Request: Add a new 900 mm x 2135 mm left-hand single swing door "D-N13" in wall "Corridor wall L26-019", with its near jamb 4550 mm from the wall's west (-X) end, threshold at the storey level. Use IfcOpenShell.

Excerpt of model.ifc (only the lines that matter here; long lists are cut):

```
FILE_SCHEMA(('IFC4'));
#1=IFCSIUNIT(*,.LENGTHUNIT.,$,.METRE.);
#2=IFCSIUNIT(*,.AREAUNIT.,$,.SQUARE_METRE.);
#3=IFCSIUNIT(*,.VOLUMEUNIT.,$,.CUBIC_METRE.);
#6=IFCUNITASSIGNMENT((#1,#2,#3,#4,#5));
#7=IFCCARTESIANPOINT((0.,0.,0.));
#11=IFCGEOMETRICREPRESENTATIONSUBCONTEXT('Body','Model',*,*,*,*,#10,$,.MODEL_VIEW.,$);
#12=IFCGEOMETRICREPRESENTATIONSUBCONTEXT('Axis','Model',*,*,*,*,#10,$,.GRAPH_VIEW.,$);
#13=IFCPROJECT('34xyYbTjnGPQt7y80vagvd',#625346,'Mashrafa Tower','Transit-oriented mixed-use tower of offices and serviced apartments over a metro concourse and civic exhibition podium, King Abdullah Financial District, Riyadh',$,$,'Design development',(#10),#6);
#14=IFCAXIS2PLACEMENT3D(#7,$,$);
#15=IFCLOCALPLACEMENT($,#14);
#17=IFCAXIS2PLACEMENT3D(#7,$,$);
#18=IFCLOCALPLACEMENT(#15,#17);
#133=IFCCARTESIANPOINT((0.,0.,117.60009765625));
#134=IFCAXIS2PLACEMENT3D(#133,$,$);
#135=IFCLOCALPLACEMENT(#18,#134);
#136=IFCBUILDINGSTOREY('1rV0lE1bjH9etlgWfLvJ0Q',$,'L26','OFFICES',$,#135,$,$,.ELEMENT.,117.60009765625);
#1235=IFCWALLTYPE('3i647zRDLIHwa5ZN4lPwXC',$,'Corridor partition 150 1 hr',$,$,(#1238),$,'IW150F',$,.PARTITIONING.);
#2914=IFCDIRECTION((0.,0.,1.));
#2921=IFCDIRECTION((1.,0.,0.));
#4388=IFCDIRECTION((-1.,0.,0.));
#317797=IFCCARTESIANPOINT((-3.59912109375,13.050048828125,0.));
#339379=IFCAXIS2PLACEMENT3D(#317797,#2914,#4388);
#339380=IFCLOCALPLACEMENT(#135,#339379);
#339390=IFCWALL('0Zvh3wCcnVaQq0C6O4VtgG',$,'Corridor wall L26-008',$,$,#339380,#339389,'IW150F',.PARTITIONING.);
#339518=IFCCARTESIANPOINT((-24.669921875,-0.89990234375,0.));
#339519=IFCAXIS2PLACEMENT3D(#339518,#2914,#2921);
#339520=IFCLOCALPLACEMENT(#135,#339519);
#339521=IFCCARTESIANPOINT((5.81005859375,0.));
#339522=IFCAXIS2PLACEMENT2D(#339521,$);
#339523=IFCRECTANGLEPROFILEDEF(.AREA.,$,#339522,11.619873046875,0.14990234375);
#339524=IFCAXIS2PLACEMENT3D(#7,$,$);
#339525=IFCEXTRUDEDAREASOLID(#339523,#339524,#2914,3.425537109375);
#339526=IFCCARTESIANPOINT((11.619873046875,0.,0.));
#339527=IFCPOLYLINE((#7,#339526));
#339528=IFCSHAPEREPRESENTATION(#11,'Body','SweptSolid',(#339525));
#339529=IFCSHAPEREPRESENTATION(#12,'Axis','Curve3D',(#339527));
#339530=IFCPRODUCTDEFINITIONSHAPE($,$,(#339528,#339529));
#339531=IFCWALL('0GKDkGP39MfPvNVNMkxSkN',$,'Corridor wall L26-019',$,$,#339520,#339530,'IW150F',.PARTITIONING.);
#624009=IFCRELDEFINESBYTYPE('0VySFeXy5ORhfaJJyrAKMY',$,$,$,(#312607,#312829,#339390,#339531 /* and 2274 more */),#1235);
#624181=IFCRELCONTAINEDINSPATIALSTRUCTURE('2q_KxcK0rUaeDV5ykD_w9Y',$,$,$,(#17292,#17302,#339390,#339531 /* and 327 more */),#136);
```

```python
import numpy as np
import ifcopenshell
import ifcopenshell.api.feature
import ifcopenshell.api.geometry
import ifcopenshell.api.root
import ifcopenshell.api.spatial
import ifcopenshell.geom
import ifcopenshell.util.element
import ifcopenshell.util.placement
import ifcopenshell.util.representation
import ifcopenshell.util.shape
import ifcopenshell.util.unit

model = ifcopenshell.open("model.ifc")
unit_scale = ifcopenshell.util.unit.calculate_unit_scale(model)
settings = ifcopenshell.geom.settings()


def volume(element):
    """Net volume in cubic metres, openings subtracted."""
    shape = ifcopenshell.geom.create_shape(settings, element)
    return ifcopenshell.util.shape.get_volume(shape.geometry)


wall = model.by_guid("0GKDkGP39MfPvNVNMkxSkN")
storey = ifcopenshell.util.element.get_container(wall, ifc_class="IfcBuildingStorey")
context = ifcopenshell.util.representation.get_context(model, "Model", "Body", "MODEL_VIEW")
before = volume(wall)

width, height, from_end, sill = 0.9, 2.135, 4.55, 0.0  # metres

# The wall runs along its own X axis, and the end named is its -X end.
wall_shape = ifcopenshell.geom.create_shape(settings, wall)
x, y, z = ifcopenshell.util.shape.get_vertices(wall_shape.geometry).T
start = x.min() + from_end
face, thickness = float(y.min()), float(y.max() - y.min())
wall_matrix = ifcopenshell.util.placement.get_local_placement(wall.ObjectPlacement)
level = ifcopenshell.util.placement.get_local_placement(storey.ObjectPlacement)[2, 3]


def in_wall(x, y):
    """Placement at x, y metres in the wall's axes, at sill height."""
    matrix = wall_matrix.copy()
    matrix[:, 3] = wall_matrix @ np.array([x / unit_scale, y / unit_scale, 0.0, 1.0])
    matrix[2, 3] = level + sill / unit_scale
    return matrix


# Opening: a box that overshoots both wall faces by 50 mm.
opening = ifcopenshell.api.root.create_entity(model, ifc_class="IfcOpeningElement", predefined_type="OPENING")
box = ifcopenshell.api.geometry.add_wall_representation(
    model, context=context, length=width, height=height, thickness=thickness + 0.1
)
ifcopenshell.api.geometry.assign_representation(model, product=opening, representation=box)
ifcopenshell.api.geometry.edit_object_placement(model, product=opening, matrix=in_wall(start, face - 0.05), is_si=False)
ifcopenshell.api.feature.add_feature(model, feature=opening, element=wall)

door = ifcopenshell.api.root.create_entity(model, ifc_class="IfcDoor", name="D-N13", predefined_type="DOOR")
door.OverallWidth, door.OverallHeight = width / unit_scale, height / unit_scale
door.OperationType = "SINGLE_SWING_LEFT"
body = ifcopenshell.api.geometry.add_door_representation(
    model,
    context=context,
    overall_width=door.OverallWidth,
    overall_height=door.OverallHeight,
    operation_type="SINGLE_SWING_LEFT",
    lining_properties={"LiningDepth": thickness / unit_scale, "ThresholdDepth": thickness / unit_scale},
)
ifcopenshell.api.geometry.assign_representation(model, product=door, representation=body)
ifcopenshell.api.spatial.assign_container(model, products=[door], relating_structure=storey)
ifcopenshell.api.feature.add_filling(model, opening=opening, element=door)

# The lining spans the wall, so the door starts at the wall face.
ifcopenshell.api.geometry.edit_object_placement(model, product=door, matrix=in_wall(start, face), is_si=False)

after = volume(wall)

print(f"wall volume {before:.3f} -> {after:.3f} m3")

model.write("model-out.ifc")
```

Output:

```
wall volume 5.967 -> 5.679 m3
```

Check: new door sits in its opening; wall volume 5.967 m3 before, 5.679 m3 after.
